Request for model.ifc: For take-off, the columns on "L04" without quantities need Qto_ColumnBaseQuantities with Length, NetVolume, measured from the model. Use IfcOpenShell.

First a look at what the model holds.

```python
import ifcopenshell
import ifcopenshell.util.element
import ifcopenshell.util.unit

model = ifcopenshell.open("model.ifc")
print(model.schema)
for unit_type in ("LENGTHUNIT", "AREAUNIT", "VOLUMEUNIT"):
    print(unit_type, ifcopenshell.util.unit.calculate_unit_scale(model, unit_type))
storey = next(s for s in model.by_type("IfcBuildingStorey") if s.Name == "L04")
columns = [e for e in ifcopenshell.util.element.get_decomposition(storey) if e.is_a("IfcColumn")]
for e in sorted(columns, key=lambda e: e.id()):
    print(e.id(), e.is_a(), e.Name, list(ifcopenshell.util.element.get_psets(e, qtos_only=True)), sep=" | ")
```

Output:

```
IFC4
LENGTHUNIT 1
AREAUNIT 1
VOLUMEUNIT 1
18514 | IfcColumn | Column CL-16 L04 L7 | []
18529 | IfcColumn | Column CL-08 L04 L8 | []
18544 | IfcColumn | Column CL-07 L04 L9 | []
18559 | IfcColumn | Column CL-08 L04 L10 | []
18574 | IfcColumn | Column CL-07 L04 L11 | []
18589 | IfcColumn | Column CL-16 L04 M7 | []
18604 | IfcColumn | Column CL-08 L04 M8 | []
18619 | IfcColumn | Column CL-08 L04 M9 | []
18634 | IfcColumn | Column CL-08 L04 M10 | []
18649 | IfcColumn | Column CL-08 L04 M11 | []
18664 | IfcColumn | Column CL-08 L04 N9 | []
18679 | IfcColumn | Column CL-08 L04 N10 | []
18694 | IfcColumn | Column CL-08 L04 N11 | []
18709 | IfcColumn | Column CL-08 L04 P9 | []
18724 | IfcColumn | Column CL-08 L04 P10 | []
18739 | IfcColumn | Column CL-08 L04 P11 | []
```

```python
import ifcopenshell
import ifcopenshell.api.pset
import ifcopenshell.geom
import ifcopenshell.util.element
import ifcopenshell.util.shape
import ifcopenshell.util.unit

model = ifcopenshell.open("model.ifc")
unit_scale = ifcopenshell.util.unit.calculate_unit_scale(model)
volume_scale = ifcopenshell.util.unit.calculate_unit_scale(model, "VOLUMEUNIT")
settings = ifcopenshell.geom.settings()

storey = next(s for s in model.by_type("IfcBuildingStorey") if s.Name == "L04")
columns = [e for e in ifcopenshell.util.element.get_decomposition(storey) if e.is_a("IfcColumn")]

for e in sorted(columns, key=lambda e: e.id()):
    if ifcopenshell.util.element.get_psets(e, qtos_only=True, should_inherit=False):
        continue
    # Geometry comes back in metres, in the element's own axes.
    shape = ifcopenshell.geom.create_shape(settings, e)
    values = {
        "Length": ifcopenshell.util.shape.get_z(shape.geometry) / unit_scale,
        "NetVolume": ifcopenshell.util.shape.get_volume(shape.geometry) / volume_scale,
    }
    qto = ifcopenshell.api.pset.add_qto(model, product=e, name="Qto_ColumnBaseQuantities")
    ifcopenshell.api.pset.edit_qto(model, qto=qto, properties=values)
    print(e.id(), {k: round(v, 3) for k, v in values.items()})

model.write("model-out.ifc")
```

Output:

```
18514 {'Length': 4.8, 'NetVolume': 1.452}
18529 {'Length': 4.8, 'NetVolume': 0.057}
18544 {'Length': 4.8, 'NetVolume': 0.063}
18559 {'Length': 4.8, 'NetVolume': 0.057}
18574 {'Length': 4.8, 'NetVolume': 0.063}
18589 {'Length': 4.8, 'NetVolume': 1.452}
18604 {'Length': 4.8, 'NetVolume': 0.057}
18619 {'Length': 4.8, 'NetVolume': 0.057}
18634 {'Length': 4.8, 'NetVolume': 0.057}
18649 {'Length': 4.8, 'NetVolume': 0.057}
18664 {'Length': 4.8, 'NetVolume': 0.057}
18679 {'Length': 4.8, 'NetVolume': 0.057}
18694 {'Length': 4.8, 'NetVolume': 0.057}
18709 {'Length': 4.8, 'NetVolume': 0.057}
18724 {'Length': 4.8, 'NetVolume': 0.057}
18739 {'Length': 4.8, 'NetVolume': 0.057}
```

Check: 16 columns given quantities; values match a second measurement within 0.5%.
